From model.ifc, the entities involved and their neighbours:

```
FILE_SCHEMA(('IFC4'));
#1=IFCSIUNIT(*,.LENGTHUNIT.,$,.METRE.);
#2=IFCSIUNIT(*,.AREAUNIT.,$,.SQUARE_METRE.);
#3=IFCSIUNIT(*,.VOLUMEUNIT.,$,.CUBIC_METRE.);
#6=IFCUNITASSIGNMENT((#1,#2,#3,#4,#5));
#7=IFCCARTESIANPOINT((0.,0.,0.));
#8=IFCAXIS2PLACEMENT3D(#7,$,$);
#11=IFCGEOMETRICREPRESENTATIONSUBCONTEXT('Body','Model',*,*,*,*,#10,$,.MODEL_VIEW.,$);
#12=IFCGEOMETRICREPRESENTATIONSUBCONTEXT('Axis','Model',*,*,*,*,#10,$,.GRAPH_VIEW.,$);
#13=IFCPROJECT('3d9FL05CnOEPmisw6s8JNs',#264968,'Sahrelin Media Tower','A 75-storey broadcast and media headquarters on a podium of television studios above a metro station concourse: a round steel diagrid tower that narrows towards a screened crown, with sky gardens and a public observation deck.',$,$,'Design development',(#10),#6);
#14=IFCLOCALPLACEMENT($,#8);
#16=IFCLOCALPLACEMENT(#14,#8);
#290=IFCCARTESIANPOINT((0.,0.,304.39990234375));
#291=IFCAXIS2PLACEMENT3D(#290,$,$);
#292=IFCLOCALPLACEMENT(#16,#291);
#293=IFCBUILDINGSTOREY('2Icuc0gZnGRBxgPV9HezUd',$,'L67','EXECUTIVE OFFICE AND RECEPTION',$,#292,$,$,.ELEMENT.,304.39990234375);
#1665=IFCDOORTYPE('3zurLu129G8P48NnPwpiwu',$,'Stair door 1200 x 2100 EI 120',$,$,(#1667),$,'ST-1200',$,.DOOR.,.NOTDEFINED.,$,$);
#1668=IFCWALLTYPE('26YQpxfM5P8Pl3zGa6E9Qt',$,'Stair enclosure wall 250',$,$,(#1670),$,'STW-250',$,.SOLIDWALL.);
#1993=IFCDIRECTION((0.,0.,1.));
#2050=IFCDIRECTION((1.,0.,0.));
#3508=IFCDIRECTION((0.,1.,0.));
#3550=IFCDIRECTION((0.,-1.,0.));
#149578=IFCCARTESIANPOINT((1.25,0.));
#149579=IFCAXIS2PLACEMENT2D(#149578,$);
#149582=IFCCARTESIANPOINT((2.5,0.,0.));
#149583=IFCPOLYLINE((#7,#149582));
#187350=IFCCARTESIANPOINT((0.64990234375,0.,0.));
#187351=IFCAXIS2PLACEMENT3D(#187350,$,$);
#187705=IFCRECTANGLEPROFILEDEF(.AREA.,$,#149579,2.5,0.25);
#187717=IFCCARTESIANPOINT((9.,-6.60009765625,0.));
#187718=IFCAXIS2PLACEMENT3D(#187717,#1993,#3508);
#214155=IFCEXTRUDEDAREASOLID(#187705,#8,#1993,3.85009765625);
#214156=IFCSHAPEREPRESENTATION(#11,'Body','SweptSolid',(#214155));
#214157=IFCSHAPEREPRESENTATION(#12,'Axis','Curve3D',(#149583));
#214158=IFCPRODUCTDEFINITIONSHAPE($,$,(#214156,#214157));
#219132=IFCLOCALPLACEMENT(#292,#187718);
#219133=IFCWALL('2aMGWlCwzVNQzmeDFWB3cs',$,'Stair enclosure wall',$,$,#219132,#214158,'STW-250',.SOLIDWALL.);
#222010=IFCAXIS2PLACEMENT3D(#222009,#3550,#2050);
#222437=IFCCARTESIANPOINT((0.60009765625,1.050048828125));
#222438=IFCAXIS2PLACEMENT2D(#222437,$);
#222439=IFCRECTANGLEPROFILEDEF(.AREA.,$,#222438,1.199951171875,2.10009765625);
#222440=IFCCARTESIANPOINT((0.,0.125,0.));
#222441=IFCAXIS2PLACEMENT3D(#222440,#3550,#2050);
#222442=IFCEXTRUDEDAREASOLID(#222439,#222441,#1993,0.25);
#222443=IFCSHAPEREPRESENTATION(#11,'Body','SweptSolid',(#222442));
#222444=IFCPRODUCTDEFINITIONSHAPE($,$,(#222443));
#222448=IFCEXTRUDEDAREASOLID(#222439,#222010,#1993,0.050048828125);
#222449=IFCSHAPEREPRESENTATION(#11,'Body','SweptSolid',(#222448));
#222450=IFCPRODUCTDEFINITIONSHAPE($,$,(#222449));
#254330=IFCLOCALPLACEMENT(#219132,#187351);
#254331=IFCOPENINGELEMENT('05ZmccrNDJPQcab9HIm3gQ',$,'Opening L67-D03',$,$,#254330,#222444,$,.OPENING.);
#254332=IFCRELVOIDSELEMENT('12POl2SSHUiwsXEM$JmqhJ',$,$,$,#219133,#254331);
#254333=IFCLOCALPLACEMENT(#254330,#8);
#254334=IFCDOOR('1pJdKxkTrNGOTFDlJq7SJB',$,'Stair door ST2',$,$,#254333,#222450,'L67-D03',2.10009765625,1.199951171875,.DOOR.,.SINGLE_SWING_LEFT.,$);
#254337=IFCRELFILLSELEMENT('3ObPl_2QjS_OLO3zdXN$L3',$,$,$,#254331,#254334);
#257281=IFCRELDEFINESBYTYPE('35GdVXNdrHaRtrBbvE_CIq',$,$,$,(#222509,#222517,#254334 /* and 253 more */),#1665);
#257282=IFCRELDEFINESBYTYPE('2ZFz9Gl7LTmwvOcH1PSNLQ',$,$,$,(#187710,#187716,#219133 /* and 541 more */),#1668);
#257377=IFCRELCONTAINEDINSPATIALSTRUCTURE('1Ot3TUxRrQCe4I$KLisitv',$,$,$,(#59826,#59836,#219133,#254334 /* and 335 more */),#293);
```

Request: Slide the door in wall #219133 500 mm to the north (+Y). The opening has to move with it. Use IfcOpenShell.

```python
import ifcopenshell
import ifcopenshell.api.geometry
import ifcopenshell.util.placement

model = ifcopenshell.open("model.ifc")

door = model.by_id(254334)
opening = door.FillsVoids[0].RelatingOpeningElement
wall = opening.VoidsElements[0].RelatingBuildingElement

wall_matrix = ifcopenshell.util.placement.get_local_placement(wall.ObjectPlacement)
shift = wall_matrix[:3, 0] * 0.5
before = ifcopenshell.util.placement.get_local_placement(door.ObjectPlacement)[:3, 3].copy()

# The door is placed relative to its opening, so it follows when the opening moves.
matrix = ifcopenshell.util.placement.get_local_placement(opening.ObjectPlacement)
matrix[:3, 3] += shift
ifcopenshell.api.geometry.edit_object_placement(
    model, product=opening, matrix=matrix, is_si=False, should_transform_children=True
)

after = ifcopenshell.util.placement.get_local_placement(door.ObjectPlacement)[:3, 3]
print("door moved by", (after - before).round(3) + 0.0)

model.write("model_updated.ifc")
```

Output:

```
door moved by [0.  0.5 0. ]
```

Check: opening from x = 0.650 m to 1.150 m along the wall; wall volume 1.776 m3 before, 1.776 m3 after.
